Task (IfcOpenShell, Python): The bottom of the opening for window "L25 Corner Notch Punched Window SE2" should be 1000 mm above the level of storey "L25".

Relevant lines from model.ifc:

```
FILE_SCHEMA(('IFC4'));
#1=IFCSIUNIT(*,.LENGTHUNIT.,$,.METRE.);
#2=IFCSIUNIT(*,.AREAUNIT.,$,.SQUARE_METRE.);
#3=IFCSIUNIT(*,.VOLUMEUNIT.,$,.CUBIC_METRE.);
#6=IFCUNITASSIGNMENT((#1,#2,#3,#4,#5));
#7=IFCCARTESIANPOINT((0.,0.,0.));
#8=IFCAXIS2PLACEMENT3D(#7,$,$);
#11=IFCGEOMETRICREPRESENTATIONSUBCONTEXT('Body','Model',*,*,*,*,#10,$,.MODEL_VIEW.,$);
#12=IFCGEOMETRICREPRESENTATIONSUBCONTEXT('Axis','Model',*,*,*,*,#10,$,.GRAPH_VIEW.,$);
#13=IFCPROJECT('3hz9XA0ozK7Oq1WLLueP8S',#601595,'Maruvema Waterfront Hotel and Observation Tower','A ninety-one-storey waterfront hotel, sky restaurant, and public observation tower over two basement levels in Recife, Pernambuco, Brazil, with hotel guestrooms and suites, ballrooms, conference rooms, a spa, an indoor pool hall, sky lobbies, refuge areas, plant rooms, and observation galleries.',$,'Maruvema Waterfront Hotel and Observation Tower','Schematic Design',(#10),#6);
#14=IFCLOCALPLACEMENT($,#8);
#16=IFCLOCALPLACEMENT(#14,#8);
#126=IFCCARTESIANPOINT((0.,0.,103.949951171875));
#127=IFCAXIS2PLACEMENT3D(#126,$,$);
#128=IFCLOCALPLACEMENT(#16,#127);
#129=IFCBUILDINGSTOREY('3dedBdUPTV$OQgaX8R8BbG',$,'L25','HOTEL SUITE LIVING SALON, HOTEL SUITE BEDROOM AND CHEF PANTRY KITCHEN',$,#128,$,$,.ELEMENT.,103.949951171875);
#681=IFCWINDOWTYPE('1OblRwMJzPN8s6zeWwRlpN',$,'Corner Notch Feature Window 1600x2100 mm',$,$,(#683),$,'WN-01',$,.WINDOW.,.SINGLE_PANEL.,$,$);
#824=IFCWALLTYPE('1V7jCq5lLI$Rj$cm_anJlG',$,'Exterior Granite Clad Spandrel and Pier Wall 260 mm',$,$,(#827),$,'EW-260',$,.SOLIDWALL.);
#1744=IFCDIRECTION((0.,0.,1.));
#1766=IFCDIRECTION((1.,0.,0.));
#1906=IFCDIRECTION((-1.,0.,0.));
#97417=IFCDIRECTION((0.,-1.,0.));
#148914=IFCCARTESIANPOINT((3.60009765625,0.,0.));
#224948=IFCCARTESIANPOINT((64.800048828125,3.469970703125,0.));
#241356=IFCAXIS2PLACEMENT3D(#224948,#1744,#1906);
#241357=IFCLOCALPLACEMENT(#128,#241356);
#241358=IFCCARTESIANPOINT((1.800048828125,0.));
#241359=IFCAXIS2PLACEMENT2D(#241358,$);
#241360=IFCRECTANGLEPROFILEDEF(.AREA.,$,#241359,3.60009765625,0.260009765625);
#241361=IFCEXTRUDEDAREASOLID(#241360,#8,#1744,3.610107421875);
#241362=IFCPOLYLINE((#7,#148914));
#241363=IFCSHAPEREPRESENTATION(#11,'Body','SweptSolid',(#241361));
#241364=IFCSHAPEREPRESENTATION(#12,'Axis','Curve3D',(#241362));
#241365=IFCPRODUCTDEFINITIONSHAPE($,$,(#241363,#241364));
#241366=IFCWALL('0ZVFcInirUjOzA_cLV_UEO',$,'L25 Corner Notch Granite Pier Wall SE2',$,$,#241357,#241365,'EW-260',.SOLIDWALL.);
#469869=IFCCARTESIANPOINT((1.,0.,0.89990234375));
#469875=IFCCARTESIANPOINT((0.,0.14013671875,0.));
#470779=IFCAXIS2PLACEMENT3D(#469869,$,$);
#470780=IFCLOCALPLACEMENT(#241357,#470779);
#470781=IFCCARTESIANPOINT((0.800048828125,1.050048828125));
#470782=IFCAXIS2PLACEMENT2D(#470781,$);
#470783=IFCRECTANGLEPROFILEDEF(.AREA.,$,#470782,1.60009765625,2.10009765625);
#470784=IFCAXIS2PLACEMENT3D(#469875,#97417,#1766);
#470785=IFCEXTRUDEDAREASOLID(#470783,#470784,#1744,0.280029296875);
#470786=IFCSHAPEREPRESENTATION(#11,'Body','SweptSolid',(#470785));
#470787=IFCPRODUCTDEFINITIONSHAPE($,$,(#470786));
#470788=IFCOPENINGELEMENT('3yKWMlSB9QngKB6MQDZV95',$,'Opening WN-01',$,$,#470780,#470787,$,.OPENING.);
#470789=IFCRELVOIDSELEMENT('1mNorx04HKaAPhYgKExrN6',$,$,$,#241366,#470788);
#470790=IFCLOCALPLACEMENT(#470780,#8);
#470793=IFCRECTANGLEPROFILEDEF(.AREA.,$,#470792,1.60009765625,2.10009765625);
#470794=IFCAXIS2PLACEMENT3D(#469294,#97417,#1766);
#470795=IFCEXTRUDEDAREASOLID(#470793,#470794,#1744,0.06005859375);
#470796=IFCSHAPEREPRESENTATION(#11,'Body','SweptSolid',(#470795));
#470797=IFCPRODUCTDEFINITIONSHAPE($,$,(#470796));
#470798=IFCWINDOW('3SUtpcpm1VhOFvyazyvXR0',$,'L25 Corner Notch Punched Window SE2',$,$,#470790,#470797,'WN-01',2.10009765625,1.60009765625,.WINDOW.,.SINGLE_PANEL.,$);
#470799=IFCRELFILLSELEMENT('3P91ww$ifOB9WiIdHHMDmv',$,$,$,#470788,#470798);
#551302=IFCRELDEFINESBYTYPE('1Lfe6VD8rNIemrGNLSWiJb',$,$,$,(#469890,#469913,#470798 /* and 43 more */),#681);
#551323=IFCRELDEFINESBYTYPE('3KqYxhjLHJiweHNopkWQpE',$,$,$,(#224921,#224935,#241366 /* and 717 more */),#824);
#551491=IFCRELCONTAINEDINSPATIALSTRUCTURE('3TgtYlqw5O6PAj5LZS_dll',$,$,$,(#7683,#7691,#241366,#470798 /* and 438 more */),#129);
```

```python
import numpy as np
import ifcopenshell
import ifcopenshell.api.geometry
import ifcopenshell.geom
import ifcopenshell.util.element
import ifcopenshell.util.placement
import ifcopenshell.util.shape
import ifcopenshell.util.unit

model = ifcopenshell.open("model.ifc")
unit_scale = ifcopenshell.util.unit.calculate_unit_scale(model)

window = model.by_guid("3SUtpcpm1VhOFvyazyvXR0")
opening = window.FillsVoids[0].RelatingOpeningElement
storey = ifcopenshell.util.element.get_container(window, ifc_class="IfcBuildingStorey")
level = ifcopenshell.util.placement.get_local_placement(storey.ObjectPlacement)[2, 3]

# The opening's origin need not be at the sill, so measure its lowest point.
shape = ifcopenshell.geom.create_shape(ifcopenshell.geom.settings(), opening)
bottom = ifcopenshell.util.shape.get_shape_bottom_elevation(shape, shape.geometry) / unit_scale
dz = level + 1 / unit_scale - bottom

shift = np.array([0.0, 0.0, dz])
# The window is placed relative to its opening, so it follows when the opening moves.
matrix = ifcopenshell.util.placement.get_local_placement(opening.ObjectPlacement)
matrix[:3, 3] += shift
ifcopenshell.api.geometry.edit_object_placement(
    model, product=opening, matrix=matrix, is_si=False, should_transform_children=True
)

print(f"moved by {dz * unit_scale:+.3f} m")

model.write("model_rev.ifc")
```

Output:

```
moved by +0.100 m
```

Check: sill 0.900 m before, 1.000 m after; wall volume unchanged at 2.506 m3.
